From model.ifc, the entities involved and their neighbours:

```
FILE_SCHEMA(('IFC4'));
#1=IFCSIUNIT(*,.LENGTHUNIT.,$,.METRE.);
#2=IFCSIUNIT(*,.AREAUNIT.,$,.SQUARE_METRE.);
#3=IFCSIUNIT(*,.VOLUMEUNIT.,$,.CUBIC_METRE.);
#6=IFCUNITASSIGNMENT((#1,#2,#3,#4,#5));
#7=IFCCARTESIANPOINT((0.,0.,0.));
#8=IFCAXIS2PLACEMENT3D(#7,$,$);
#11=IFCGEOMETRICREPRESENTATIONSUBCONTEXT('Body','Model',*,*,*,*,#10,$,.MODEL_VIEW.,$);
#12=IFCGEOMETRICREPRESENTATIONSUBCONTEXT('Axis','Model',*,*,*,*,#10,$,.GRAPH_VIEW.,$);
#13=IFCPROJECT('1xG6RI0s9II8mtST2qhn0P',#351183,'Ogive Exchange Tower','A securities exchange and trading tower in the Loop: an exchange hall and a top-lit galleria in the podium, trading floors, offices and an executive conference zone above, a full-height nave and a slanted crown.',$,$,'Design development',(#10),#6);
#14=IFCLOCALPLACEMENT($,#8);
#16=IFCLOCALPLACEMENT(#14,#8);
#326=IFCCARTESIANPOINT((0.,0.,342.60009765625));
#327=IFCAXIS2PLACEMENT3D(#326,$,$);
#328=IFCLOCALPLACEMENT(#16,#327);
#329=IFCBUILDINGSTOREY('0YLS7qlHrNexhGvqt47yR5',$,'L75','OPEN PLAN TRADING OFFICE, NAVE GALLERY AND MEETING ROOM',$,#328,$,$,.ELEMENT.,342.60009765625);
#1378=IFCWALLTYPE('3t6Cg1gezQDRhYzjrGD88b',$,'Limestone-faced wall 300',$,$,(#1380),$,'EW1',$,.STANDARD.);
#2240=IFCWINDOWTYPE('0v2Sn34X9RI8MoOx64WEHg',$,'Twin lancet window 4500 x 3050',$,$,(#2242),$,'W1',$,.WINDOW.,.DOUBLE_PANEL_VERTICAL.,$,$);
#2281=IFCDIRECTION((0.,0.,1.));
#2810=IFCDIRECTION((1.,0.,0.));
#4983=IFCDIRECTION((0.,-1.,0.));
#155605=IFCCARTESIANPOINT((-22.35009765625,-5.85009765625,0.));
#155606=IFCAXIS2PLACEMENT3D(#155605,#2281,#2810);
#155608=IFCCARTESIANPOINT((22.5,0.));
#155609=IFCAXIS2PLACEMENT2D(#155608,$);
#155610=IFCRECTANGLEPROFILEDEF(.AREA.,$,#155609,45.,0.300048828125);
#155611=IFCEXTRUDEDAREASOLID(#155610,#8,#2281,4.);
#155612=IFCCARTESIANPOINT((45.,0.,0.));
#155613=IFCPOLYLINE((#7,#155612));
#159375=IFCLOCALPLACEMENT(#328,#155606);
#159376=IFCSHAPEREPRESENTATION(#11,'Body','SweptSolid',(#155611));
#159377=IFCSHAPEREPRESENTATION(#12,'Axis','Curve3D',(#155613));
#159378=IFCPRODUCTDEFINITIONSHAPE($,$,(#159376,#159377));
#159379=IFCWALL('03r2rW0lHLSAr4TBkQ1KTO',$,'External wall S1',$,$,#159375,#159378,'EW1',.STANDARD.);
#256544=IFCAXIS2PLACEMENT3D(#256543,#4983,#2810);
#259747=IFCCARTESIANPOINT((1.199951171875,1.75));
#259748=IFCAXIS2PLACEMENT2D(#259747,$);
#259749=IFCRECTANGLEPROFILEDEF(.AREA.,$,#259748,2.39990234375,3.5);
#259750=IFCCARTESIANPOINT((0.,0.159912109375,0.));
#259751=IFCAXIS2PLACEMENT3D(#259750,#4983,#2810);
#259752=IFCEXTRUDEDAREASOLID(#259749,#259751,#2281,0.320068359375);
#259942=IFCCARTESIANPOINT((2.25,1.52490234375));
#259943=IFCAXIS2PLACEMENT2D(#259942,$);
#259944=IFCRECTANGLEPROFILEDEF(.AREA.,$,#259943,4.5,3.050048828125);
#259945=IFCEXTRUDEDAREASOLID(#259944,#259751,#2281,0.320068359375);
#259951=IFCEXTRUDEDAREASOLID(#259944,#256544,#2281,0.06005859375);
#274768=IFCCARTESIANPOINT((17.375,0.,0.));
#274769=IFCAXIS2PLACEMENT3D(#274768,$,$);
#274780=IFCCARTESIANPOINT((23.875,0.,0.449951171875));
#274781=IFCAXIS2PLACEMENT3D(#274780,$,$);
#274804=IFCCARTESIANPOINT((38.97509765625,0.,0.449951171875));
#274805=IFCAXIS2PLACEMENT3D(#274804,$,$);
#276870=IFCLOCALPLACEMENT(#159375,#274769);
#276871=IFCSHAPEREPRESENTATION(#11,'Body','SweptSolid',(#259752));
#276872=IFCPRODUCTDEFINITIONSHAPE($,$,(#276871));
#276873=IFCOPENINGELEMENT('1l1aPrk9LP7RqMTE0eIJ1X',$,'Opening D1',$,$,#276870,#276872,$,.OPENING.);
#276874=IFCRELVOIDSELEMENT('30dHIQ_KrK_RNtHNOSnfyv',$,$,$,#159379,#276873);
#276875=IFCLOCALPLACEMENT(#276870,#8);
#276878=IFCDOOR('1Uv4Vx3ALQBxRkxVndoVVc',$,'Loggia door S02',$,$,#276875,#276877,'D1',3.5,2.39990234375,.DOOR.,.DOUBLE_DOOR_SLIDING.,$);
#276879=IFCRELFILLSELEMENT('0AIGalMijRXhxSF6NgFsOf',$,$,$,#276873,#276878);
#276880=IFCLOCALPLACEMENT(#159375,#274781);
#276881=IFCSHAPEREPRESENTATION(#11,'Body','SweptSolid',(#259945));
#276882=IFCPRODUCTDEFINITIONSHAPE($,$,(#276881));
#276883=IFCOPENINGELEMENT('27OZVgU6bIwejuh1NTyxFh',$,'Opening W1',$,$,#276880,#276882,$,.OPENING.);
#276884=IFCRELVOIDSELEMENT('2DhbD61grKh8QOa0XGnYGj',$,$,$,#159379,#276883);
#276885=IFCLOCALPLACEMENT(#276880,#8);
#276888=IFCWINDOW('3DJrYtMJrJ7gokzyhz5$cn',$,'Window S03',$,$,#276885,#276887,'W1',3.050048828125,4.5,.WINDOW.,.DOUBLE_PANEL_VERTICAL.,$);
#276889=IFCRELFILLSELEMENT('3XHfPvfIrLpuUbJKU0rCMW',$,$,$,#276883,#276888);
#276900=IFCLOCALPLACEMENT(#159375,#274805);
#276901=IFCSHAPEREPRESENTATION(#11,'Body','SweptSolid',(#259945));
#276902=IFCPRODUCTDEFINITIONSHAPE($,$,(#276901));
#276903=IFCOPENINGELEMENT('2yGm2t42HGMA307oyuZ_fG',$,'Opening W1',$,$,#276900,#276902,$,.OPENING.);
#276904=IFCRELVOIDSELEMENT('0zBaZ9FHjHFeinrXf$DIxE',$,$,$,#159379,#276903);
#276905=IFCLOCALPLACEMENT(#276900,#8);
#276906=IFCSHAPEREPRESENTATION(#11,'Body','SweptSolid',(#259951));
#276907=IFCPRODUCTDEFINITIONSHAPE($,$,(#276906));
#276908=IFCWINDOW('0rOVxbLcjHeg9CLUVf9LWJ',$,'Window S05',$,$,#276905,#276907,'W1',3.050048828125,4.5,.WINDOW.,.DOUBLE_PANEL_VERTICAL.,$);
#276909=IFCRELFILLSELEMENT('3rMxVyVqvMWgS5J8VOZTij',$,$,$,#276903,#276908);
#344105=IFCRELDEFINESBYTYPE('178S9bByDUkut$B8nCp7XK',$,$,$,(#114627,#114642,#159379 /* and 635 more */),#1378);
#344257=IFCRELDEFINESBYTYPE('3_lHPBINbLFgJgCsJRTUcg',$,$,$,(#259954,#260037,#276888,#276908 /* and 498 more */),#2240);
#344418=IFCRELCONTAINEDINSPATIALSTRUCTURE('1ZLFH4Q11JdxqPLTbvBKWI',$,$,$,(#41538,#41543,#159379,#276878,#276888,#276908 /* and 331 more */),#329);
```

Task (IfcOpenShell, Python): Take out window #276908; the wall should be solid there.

```python
import ifcopenshell
import ifcopenshell.api.feature
import ifcopenshell.api.root
import ifcopenshell.geom
import ifcopenshell.util.shape

model = ifcopenshell.open("model.ifc")
settings = ifcopenshell.geom.settings()


def volume(element):
    """Net volume in cubic metres, openings subtracted."""
    shape = ifcopenshell.geom.create_shape(settings, element)
    return ifcopenshell.util.shape.get_volume(shape.geometry)


window = model.by_id(276908)
opening = window.FillsVoids[0].RelatingOpeningElement
wall = opening.VoidsElements[0].RelatingBuildingElement
before = volume(wall)

ifcopenshell.api.root.remove_product(model, product=window)
ifcopenshell.api.feature.remove_feature(model, feature=opening)

after = volume(wall)

print(f"wall volume {before:.3f} -> {after:.3f} m3")

model.write("model-out.ifc")
```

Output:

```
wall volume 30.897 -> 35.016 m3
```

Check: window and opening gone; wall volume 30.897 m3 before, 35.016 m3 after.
